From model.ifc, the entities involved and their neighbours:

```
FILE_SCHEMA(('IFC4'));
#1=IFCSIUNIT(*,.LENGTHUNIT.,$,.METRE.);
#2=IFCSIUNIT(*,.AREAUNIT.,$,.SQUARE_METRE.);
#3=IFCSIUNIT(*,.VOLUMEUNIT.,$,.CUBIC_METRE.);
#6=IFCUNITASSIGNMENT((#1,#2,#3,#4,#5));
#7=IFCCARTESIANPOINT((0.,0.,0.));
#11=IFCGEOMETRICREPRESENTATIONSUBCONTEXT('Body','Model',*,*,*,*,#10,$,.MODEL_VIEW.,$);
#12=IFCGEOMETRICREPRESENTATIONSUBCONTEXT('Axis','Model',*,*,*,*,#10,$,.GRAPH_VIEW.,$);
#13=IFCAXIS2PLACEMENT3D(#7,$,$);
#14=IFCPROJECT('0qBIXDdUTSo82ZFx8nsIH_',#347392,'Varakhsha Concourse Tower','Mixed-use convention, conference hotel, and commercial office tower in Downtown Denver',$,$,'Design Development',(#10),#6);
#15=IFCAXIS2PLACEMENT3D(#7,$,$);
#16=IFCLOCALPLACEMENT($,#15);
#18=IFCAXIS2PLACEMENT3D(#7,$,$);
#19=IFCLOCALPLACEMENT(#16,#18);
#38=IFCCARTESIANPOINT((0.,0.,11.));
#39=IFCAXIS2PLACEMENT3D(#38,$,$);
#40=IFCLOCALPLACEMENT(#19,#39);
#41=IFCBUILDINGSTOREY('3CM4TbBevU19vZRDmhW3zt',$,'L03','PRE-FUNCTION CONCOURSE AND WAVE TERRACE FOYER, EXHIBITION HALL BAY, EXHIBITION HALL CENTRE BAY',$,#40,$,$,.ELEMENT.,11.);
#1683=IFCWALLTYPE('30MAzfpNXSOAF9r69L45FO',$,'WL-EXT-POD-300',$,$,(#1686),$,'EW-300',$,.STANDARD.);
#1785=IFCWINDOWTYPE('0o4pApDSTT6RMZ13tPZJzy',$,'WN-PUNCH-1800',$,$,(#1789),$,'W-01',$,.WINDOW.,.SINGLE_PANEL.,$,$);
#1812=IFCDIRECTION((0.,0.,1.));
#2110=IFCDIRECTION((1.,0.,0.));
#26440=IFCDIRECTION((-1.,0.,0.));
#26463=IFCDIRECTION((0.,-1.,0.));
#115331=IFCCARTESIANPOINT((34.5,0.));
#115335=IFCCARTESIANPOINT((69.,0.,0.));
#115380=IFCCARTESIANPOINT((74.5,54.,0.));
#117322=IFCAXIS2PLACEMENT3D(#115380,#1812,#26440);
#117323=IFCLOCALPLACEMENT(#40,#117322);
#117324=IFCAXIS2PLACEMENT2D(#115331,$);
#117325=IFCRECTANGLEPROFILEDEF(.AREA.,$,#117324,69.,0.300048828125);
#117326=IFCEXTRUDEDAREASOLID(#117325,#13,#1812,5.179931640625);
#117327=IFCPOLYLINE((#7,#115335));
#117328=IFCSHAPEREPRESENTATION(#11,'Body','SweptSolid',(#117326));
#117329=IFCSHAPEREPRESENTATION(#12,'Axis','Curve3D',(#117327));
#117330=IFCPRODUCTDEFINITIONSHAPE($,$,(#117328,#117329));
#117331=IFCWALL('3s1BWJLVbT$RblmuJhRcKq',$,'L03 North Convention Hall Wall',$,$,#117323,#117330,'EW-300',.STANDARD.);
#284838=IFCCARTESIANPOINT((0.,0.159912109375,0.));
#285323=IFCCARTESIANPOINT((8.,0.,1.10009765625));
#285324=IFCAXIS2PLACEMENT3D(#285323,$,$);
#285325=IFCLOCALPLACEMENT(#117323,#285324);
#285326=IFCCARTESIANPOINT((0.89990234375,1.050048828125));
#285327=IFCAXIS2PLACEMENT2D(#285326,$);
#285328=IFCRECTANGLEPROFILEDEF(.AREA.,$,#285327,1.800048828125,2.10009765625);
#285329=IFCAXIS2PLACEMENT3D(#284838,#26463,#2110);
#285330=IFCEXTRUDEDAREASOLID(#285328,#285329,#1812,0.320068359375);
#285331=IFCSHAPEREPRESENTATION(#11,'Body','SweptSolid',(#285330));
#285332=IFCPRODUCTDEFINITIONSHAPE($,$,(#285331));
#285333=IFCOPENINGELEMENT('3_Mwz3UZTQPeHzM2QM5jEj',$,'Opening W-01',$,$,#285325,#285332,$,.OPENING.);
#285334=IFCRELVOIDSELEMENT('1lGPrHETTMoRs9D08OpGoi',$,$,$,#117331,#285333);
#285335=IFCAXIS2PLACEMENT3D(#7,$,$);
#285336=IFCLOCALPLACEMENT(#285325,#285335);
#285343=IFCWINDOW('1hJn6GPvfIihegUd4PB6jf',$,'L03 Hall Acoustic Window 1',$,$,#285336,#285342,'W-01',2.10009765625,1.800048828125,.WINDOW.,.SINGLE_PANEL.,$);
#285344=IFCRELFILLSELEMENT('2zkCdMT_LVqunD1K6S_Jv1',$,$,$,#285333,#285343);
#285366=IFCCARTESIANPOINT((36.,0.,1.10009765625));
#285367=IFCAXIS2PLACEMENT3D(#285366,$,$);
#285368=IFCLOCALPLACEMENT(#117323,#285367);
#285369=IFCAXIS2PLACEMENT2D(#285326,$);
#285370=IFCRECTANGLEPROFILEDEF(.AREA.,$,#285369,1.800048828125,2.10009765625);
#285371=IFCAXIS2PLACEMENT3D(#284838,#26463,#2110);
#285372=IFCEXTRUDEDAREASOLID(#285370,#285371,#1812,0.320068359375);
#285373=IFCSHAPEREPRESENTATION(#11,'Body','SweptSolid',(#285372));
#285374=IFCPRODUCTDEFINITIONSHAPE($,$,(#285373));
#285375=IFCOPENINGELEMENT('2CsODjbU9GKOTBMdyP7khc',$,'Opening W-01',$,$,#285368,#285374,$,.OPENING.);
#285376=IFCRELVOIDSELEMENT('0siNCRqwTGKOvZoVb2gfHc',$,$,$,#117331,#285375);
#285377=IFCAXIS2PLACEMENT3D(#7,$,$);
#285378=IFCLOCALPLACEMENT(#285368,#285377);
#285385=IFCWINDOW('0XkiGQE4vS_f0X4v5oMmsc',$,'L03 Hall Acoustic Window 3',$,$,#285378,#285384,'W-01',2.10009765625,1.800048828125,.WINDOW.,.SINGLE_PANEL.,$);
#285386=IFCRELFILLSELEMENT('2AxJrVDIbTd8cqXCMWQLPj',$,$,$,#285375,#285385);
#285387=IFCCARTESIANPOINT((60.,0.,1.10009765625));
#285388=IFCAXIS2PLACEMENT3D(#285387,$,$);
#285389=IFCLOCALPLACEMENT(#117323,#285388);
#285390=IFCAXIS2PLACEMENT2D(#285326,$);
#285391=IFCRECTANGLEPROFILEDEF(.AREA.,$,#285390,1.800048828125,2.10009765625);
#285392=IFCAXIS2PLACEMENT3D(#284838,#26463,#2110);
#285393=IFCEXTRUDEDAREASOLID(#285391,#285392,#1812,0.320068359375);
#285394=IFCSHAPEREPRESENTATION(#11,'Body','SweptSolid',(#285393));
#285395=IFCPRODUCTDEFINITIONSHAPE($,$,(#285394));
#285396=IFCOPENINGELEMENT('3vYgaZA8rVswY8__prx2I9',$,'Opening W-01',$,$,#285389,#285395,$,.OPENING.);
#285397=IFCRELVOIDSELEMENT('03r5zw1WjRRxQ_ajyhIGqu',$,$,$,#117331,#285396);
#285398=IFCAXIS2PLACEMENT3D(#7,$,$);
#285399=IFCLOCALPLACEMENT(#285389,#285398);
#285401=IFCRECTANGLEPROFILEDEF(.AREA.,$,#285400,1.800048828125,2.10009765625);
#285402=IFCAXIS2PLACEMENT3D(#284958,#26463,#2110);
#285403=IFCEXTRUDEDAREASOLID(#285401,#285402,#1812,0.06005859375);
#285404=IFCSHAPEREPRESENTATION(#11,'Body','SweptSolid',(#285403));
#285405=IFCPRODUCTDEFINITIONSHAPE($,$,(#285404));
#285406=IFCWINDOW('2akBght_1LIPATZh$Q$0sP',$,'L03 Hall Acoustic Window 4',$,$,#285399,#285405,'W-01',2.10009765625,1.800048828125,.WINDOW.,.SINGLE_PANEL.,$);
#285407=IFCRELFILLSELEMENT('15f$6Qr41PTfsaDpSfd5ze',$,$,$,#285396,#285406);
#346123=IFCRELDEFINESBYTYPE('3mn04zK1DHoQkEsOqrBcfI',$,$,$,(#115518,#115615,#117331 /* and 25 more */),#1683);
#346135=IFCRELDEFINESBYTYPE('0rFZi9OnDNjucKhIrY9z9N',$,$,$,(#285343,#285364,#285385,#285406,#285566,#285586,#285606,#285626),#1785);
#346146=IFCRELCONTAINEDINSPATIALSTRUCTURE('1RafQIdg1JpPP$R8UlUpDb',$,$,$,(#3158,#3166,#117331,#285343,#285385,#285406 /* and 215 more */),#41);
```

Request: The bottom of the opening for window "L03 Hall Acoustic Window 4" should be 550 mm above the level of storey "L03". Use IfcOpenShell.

```python
import numpy as np
import ifcopenshell
import ifcopenshell.api.geometry
import ifcopenshell.geom
import ifcopenshell.util.element
import ifcopenshell.util.placement
import ifcopenshell.util.shape
import ifcopenshell.util.unit

model = ifcopenshell.open("model.ifc")
unit_scale = ifcopenshell.util.unit.calculate_unit_scale(model)

window = model.by_guid("2akBght_1LIPATZh$Q$0sP")
opening = window.FillsVoids[0].RelatingOpeningElement
storey = ifcopenshell.util.element.get_container(window, ifc_class="IfcBuildingStorey")
level = ifcopenshell.util.placement.get_local_placement(storey.ObjectPlacement)[2, 3]

# The opening's origin need not be at the sill, so measure its lowest point.
shape = ifcopenshell.geom.create_shape(ifcopenshell.geom.settings(), opening)
bottom = ifcopenshell.util.shape.get_shape_bottom_elevation(shape, shape.geometry) / unit_scale
dz = level + 0.55 - bottom

shift = np.array([0.0, 0.0, dz])
# The window is placed relative to its opening, so it follows when the opening moves.
matrix = ifcopenshell.util.placement.get_local_placement(opening.ObjectPlacement)
matrix[:3, 3] += shift
ifcopenshell.api.geometry.edit_object_placement(
    model, product=opening, matrix=matrix, is_si=False, should_transform_children=True
)

print(f"moved by {dz * unit_scale:+.3f} m")

model.write("model_v2.ifc")
```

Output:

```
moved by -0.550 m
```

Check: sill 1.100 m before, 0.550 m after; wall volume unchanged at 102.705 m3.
